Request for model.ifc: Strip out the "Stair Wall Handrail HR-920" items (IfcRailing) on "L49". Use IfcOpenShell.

First a look at what the model holds.

```python
import ifcopenshell
import ifcopenshell.util.element

model = ifcopenshell.open("model.ifc")
print(model.schema)
storey = next(s for s in model.by_type("IfcBuildingStorey") if s.Name == "L49")
railings = [e for e in ifcopenshell.util.element.get_decomposition(storey) if e.is_a("IfcRailing")]
seen = {}
for e in railings:
    element_type = ifcopenshell.util.element.get_type(e)
    name = element_type.Name if element_type not in (None, e) else None
    seen[name] = seen.get(name, 0) + 1
for name, count in sorted(seen.items(), key=str):
    print(count, "x", name)
```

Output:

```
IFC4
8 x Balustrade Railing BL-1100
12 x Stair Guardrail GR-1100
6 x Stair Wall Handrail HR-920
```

```python
import ifcopenshell
import ifcopenshell.api.root
import ifcopenshell.util.element

model = ifcopenshell.open("model.ifc")

storey = next(s for s in model.by_type("IfcBuildingStorey") if s.Name == "L49")
railings = [e for e in ifcopenshell.util.element.get_decomposition(storey) if e.is_a("IfcRailing")]
targets = [e for e in railings if (t := ifcopenshell.util.element.get_type(e)) not in (None, e) and t.Name == "Stair Wall Handrail HR-920"]

for e in targets:
    ifcopenshell.api.root.remove_product(model, product=e)
print(len(targets), "removed")

model.write("model-out.ifc")
```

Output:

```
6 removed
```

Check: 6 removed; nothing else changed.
